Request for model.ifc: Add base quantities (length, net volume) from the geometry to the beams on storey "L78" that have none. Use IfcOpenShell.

First a look at what the model holds.

```python
import ifcopenshell
import ifcopenshell.util.element
import ifcopenshell.util.unit

model = ifcopenshell.open("model.ifc")
print(model.schema)
for unit_type in ("LENGTHUNIT", "AREAUNIT", "VOLUMEUNIT"):
    print(unit_type, ifcopenshell.util.unit.calculate_unit_scale(model, unit_type))
storey = next(s for s in model.by_type("IfcBuildingStorey") if s.Name == "L78")
beams = [e for e in ifcopenshell.util.element.get_decomposition(storey) if e.is_a("IfcBeam")]
for e in sorted(beams, key=lambda e: e.id()):
    print(e.id(), e.is_a(), e.Name, list(ifcopenshell.util.element.get_psets(e, qtos_only=True)), sep=" | ")
```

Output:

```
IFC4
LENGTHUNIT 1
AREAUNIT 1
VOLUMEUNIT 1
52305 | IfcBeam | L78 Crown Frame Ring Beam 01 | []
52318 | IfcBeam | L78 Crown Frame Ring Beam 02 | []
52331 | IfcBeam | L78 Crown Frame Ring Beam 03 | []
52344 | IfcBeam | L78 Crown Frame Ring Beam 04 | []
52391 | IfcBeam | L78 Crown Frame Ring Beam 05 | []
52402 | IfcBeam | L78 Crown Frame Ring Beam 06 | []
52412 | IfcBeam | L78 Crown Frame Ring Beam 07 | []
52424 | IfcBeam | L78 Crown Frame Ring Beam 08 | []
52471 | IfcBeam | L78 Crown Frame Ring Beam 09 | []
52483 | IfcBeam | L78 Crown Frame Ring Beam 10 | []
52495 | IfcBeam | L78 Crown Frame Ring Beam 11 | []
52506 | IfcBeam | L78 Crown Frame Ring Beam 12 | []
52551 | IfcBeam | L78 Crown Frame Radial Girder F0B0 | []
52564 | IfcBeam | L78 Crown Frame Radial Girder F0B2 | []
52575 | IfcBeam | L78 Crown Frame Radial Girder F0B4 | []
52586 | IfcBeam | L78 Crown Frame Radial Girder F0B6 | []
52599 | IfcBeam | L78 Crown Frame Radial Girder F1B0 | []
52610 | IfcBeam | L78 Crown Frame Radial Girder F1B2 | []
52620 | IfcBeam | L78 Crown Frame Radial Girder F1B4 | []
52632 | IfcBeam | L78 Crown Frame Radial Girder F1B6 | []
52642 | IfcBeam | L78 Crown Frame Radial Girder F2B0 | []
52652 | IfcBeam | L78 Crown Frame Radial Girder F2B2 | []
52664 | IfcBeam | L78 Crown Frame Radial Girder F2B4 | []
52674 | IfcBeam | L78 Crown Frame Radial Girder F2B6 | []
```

```python
import ifcopenshell
import ifcopenshell.api.pset
import ifcopenshell.geom
import ifcopenshell.util.element
import ifcopenshell.util.shape
import ifcopenshell.util.unit

model = ifcopenshell.open("model.ifc")
unit_scale = ifcopenshell.util.unit.calculate_unit_scale(model)
volume_scale = ifcopenshell.util.unit.calculate_unit_scale(model, "VOLUMEUNIT")
settings = ifcopenshell.geom.settings()

storey = next(s for s in model.by_type("IfcBuildingStorey") if s.Name == "L78")
beams = [e for e in ifcopenshell.util.element.get_decomposition(storey) if e.is_a("IfcBeam")]

for e in sorted(beams, key=lambda e: e.id()):
    if ifcopenshell.util.element.get_psets(e, qtos_only=True, should_inherit=False):
        continue
    # Geometry comes back in metres, in the element's own axes.
    shape = ifcopenshell.geom.create_shape(settings, e)
    values = {
        "Length": ifcopenshell.util.shape.get_max_xyz(shape.geometry) / unit_scale,
        "NetVolume": ifcopenshell.util.shape.get_volume(shape.geometry) / volume_scale,
    }
    qto = ifcopenshell.api.pset.add_qto(model, product=e, name="Qto_BeamBaseQuantities")
    ifcopenshell.api.pset.edit_qto(model, qto=qto, properties=values)
    print(e.id(), {k: round(v, 3) for k, v in values.items()})

model.write("model_edited.ifc")
```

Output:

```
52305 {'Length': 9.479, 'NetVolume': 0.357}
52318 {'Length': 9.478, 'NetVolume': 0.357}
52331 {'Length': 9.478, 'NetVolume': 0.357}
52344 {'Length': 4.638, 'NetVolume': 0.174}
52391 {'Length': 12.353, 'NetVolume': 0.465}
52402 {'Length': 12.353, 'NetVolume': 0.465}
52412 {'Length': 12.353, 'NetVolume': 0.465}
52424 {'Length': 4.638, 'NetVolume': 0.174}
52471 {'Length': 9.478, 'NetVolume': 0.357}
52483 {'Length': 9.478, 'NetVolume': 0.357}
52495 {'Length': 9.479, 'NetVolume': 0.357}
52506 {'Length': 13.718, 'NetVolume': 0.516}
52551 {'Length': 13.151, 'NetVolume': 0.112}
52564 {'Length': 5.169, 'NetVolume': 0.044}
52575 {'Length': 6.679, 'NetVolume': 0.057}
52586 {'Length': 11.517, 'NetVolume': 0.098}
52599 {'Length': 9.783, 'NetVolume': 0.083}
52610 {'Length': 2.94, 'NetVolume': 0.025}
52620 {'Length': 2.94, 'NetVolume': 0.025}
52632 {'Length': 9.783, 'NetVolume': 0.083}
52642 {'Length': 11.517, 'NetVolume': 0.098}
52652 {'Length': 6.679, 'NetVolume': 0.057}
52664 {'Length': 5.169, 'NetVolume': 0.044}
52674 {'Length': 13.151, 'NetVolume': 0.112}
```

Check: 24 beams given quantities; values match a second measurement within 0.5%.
